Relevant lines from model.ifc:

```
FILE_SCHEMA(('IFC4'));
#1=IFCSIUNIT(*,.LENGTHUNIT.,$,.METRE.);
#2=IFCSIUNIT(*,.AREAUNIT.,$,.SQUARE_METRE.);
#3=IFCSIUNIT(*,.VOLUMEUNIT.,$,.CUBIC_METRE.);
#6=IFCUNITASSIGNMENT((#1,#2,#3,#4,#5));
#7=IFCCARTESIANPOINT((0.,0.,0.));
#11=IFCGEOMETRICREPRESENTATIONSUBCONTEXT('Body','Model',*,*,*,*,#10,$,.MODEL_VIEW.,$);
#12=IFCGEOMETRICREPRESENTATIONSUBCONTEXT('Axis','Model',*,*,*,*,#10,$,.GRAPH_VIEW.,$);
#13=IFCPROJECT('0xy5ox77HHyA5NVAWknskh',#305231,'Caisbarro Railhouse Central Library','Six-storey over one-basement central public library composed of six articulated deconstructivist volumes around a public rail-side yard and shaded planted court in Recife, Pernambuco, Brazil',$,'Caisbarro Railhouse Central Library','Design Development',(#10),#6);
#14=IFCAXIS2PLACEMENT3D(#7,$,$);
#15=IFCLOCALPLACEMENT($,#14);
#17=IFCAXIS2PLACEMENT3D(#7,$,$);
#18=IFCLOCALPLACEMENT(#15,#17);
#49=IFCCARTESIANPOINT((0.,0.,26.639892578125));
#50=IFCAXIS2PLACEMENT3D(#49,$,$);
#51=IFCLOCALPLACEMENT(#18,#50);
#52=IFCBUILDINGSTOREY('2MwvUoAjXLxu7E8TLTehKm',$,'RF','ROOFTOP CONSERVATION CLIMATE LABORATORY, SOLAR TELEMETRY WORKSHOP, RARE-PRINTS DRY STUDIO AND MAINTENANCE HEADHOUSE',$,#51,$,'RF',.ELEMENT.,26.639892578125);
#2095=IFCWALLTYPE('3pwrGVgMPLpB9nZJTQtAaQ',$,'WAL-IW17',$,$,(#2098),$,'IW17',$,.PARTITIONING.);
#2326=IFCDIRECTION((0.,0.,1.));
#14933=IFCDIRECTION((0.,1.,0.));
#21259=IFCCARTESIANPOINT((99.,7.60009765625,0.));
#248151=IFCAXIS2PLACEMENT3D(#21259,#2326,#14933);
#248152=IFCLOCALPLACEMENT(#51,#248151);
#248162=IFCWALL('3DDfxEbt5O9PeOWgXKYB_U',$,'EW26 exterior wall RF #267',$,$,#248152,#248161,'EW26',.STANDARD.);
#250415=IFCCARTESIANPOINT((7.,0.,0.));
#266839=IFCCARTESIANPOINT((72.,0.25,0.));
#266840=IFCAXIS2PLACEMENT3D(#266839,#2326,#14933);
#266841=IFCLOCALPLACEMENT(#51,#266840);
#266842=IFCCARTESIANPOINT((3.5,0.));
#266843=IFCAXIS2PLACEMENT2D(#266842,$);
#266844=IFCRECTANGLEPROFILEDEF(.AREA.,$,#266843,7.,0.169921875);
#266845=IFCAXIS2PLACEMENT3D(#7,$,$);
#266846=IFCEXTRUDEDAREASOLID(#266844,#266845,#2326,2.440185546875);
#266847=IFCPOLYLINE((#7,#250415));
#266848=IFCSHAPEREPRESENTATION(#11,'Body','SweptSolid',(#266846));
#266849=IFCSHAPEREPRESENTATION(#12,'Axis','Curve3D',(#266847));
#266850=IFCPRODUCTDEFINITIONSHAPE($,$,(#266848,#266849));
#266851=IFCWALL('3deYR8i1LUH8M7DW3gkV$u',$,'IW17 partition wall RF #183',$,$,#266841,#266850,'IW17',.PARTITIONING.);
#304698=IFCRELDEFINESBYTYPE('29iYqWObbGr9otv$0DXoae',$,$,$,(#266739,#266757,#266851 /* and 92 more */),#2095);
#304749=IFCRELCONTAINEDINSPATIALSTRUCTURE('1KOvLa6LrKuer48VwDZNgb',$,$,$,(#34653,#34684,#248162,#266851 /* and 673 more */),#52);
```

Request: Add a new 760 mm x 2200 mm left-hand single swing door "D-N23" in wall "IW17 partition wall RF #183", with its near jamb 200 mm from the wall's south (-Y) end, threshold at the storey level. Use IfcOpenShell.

```python
import numpy as np
import ifcopenshell
import ifcopenshell.api.feature
import ifcopenshell.api.geometry
import ifcopenshell.api.root
import ifcopenshell.api.spatial
import ifcopenshell.geom
import ifcopenshell.util.element
import ifcopenshell.util.placement
import ifcopenshell.util.representation
import ifcopenshell.util.shape
import ifcopenshell.util.unit

model = ifcopenshell.open("model.ifc")
unit_scale = ifcopenshell.util.unit.calculate_unit_scale(model)
settings = ifcopenshell.geom.settings()


def volume(element):
    """Net volume in cubic metres, openings subtracted."""
    shape = ifcopenshell.geom.create_shape(settings, element)
    return ifcopenshell.util.shape.get_volume(shape.geometry)


wall = model.by_guid("3deYR8i1LUH8M7DW3gkV$u")
storey = ifcopenshell.util.element.get_container(wall, ifc_class="IfcBuildingStorey")
context = ifcopenshell.util.representation.get_context(model, "Model", "Body", "MODEL_VIEW")
before = volume(wall)

width, height, from_end, sill = 0.76, 2.2, 0.2, 0.0  # metres

# The wall runs along its own X axis, and the end named is its -X end.
wall_shape = ifcopenshell.geom.create_shape(settings, wall)
x, y, z = ifcopenshell.util.shape.get_vertices(wall_shape.geometry).T
start = x.min() + from_end
face, thickness = float(y.min()), float(y.max() - y.min())
wall_matrix = ifcopenshell.util.placement.get_local_placement(wall.ObjectPlacement)
level = ifcopenshell.util.placement.get_local_placement(storey.ObjectPlacement)[2, 3]


def in_wall(x, y):
    """Placement at x, y metres in the wall's axes, at sill height."""
    matrix = wall_matrix.copy()
    matrix[:, 3] = wall_matrix @ np.array([x / unit_scale, y / unit_scale, 0.0, 1.0])
    matrix[2, 3] = level + sill / unit_scale
    return matrix


# Opening: a box that overshoots both wall faces by 50 mm.
opening = ifcopenshell.api.root.create_entity(model, ifc_class="IfcOpeningElement", predefined_type="OPENING")
box = ifcopenshell.api.geometry.add_wall_representation(
    model, context=context, length=width, height=height, thickness=thickness + 0.1
)
ifcopenshell.api.geometry.assign_representation(model, product=opening, representation=box)
ifcopenshell.api.geometry.edit_object_placement(model, product=opening, matrix=in_wall(start, face - 0.05), is_si=False)
ifcopenshell.api.feature.add_feature(model, feature=opening, element=wall)

door = ifcopenshell.api.root.create_entity(model, ifc_class="IfcDoor", name="D-N23", predefined_type="DOOR")
door.OverallWidth, door.OverallHeight = width / unit_scale, height / unit_scale
door.OperationType = "SINGLE_SWING_LEFT"
body = ifcopenshell.api.geometry.add_door_representation(
    model,
    context=context,
    overall_width=door.OverallWidth,
    overall_height=door.OverallHeight,
    operation_type="SINGLE_SWING_LEFT",
    lining_properties={"LiningDepth": thickness / unit_scale, "ThresholdDepth": thickness / unit_scale},
)
ifcopenshell.api.geometry.assign_representation(model, product=door, representation=body)
ifcopenshell.api.spatial.assign_container(model, products=[door], relating_structure=storey)
ifcopenshell.api.feature.add_filling(model, opening=opening, element=door)

# The lining spans the wall, so the door starts at the wall face.
ifcopenshell.api.geometry.edit_object_placement(model, product=door, matrix=in_wall(start, face), is_si=False)

after = volume(wall)

print(f"wall volume {before:.3f} -> {after:.3f} m3")

model.write("model_rev.ifc")
```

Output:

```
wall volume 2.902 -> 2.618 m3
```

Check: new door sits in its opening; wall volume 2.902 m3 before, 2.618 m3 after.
